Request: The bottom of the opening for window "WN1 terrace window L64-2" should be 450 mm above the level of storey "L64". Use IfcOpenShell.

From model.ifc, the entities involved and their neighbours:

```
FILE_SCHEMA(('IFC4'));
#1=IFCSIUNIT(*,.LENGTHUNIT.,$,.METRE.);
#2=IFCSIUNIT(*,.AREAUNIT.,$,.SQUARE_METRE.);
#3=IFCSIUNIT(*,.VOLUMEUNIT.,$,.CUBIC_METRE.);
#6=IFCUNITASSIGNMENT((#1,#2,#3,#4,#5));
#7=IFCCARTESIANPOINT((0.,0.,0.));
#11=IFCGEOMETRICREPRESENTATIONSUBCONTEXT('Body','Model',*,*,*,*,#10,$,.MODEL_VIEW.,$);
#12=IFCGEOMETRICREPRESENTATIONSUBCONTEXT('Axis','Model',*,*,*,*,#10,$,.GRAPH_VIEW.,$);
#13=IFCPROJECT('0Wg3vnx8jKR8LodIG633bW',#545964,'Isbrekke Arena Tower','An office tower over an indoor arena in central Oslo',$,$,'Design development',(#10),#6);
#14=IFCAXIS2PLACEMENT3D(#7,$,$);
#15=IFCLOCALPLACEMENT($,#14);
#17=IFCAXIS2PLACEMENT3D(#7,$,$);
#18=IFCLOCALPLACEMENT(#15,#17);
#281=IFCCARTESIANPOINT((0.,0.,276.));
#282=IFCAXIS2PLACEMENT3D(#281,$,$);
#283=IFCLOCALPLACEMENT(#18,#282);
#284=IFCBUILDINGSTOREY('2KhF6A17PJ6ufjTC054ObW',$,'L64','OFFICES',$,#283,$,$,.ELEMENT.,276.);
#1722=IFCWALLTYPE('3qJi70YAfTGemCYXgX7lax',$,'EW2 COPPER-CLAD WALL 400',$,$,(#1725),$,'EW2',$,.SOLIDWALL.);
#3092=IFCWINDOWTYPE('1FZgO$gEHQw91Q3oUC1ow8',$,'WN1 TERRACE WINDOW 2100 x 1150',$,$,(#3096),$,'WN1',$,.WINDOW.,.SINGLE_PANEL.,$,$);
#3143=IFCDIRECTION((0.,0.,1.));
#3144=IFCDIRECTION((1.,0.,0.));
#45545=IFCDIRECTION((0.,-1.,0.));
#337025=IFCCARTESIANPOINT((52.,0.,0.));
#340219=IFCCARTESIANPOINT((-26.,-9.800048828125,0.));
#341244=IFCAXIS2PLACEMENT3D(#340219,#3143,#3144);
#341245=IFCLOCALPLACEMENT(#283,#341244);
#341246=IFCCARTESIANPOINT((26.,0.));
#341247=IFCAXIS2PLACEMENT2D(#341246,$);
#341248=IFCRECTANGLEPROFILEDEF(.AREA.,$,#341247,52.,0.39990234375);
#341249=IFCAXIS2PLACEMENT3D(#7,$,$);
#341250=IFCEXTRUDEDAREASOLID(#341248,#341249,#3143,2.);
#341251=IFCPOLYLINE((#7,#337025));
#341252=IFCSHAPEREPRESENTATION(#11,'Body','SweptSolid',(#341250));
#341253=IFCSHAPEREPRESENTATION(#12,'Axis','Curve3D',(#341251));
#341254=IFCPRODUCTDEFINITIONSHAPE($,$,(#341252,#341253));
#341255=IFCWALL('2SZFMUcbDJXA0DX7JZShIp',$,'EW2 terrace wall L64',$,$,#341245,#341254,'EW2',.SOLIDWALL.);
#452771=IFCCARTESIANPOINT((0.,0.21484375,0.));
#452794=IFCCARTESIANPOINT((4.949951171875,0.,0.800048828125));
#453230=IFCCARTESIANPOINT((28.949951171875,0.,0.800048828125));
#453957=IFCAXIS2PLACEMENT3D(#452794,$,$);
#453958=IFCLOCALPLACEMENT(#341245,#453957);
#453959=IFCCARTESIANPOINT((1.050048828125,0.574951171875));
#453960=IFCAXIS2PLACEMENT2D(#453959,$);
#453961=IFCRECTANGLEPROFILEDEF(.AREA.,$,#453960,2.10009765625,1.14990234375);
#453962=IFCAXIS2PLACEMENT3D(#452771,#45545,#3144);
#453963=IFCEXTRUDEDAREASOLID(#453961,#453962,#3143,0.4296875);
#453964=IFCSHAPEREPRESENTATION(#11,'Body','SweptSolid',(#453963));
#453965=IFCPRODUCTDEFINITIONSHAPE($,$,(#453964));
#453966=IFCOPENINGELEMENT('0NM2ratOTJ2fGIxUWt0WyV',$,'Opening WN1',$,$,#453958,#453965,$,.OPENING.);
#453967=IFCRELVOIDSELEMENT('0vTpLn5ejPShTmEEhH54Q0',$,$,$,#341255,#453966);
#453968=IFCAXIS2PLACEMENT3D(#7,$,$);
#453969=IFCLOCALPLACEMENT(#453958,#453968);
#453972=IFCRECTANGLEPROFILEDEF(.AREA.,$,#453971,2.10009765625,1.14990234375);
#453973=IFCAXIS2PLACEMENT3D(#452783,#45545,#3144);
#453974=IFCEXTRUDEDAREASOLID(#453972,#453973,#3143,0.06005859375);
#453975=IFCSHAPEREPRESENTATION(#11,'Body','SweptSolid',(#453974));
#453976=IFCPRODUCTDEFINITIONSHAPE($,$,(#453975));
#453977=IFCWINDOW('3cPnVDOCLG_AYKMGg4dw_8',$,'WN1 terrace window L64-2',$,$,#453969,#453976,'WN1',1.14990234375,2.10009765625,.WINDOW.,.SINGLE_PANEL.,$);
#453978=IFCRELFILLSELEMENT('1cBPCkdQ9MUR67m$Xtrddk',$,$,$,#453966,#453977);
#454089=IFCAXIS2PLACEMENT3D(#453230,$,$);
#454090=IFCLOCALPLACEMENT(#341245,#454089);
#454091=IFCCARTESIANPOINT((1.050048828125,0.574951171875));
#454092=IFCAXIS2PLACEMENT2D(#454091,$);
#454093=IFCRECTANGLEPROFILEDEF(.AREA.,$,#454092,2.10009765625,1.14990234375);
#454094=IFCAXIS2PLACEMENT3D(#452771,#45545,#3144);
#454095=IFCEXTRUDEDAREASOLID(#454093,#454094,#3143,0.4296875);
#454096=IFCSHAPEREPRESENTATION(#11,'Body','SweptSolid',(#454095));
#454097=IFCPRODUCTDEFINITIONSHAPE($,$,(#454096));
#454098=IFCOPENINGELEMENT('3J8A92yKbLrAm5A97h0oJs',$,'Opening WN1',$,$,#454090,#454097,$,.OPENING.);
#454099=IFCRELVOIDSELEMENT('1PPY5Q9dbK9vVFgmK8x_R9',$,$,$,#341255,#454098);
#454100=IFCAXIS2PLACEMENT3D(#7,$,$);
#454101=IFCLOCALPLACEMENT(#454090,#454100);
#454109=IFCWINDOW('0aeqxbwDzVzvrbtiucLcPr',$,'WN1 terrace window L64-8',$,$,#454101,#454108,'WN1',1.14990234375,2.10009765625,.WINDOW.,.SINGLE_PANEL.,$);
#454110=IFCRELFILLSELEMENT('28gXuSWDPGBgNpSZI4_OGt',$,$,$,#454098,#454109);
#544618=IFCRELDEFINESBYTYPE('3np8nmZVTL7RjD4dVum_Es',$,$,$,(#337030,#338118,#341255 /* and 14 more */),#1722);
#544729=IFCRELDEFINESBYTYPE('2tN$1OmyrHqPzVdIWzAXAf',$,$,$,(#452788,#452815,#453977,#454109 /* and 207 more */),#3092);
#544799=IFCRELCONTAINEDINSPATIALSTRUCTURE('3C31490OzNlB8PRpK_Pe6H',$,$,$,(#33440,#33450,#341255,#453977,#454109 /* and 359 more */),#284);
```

```python
import numpy as np
import ifcopenshell
import ifcopenshell.api.geometry
import ifcopenshell.geom
import ifcopenshell.util.element
import ifcopenshell.util.placement
import ifcopenshell.util.shape
import ifcopenshell.util.unit

model = ifcopenshell.open("model.ifc")
unit_scale = ifcopenshell.util.unit.calculate_unit_scale(model)

window = model.by_id(453977)
opening = window.FillsVoids[0].RelatingOpeningElement
storey = ifcopenshell.util.element.get_container(window, ifc_class="IfcBuildingStorey")
level = ifcopenshell.util.placement.get_local_placement(storey.ObjectPlacement)[2, 3]

# The opening's origin need not be at the sill, so measure its lowest point.
shape = ifcopenshell.geom.create_shape(ifcopenshell.geom.settings(), opening)
bottom = ifcopenshell.util.shape.get_shape_bottom_elevation(shape, shape.geometry) / unit_scale
dz = level + 0.45 / unit_scale - bottom

shift = np.array([0.0, 0.0, dz])
# The window is placed relative to its opening, so it follows when the opening moves.
matrix = ifcopenshell.util.placement.get_local_placement(opening.ObjectPlacement)
matrix[:3, 3] += shift
ifcopenshell.api.geometry.edit_object_placement(
    model, product=opening, matrix=matrix, is_si=False, should_transform_children=True
)

print(f"moved by {dz * unit_scale:+.3f} m")

model.write("model_updated.ifc")
```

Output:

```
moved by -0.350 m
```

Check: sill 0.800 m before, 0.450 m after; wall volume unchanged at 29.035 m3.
